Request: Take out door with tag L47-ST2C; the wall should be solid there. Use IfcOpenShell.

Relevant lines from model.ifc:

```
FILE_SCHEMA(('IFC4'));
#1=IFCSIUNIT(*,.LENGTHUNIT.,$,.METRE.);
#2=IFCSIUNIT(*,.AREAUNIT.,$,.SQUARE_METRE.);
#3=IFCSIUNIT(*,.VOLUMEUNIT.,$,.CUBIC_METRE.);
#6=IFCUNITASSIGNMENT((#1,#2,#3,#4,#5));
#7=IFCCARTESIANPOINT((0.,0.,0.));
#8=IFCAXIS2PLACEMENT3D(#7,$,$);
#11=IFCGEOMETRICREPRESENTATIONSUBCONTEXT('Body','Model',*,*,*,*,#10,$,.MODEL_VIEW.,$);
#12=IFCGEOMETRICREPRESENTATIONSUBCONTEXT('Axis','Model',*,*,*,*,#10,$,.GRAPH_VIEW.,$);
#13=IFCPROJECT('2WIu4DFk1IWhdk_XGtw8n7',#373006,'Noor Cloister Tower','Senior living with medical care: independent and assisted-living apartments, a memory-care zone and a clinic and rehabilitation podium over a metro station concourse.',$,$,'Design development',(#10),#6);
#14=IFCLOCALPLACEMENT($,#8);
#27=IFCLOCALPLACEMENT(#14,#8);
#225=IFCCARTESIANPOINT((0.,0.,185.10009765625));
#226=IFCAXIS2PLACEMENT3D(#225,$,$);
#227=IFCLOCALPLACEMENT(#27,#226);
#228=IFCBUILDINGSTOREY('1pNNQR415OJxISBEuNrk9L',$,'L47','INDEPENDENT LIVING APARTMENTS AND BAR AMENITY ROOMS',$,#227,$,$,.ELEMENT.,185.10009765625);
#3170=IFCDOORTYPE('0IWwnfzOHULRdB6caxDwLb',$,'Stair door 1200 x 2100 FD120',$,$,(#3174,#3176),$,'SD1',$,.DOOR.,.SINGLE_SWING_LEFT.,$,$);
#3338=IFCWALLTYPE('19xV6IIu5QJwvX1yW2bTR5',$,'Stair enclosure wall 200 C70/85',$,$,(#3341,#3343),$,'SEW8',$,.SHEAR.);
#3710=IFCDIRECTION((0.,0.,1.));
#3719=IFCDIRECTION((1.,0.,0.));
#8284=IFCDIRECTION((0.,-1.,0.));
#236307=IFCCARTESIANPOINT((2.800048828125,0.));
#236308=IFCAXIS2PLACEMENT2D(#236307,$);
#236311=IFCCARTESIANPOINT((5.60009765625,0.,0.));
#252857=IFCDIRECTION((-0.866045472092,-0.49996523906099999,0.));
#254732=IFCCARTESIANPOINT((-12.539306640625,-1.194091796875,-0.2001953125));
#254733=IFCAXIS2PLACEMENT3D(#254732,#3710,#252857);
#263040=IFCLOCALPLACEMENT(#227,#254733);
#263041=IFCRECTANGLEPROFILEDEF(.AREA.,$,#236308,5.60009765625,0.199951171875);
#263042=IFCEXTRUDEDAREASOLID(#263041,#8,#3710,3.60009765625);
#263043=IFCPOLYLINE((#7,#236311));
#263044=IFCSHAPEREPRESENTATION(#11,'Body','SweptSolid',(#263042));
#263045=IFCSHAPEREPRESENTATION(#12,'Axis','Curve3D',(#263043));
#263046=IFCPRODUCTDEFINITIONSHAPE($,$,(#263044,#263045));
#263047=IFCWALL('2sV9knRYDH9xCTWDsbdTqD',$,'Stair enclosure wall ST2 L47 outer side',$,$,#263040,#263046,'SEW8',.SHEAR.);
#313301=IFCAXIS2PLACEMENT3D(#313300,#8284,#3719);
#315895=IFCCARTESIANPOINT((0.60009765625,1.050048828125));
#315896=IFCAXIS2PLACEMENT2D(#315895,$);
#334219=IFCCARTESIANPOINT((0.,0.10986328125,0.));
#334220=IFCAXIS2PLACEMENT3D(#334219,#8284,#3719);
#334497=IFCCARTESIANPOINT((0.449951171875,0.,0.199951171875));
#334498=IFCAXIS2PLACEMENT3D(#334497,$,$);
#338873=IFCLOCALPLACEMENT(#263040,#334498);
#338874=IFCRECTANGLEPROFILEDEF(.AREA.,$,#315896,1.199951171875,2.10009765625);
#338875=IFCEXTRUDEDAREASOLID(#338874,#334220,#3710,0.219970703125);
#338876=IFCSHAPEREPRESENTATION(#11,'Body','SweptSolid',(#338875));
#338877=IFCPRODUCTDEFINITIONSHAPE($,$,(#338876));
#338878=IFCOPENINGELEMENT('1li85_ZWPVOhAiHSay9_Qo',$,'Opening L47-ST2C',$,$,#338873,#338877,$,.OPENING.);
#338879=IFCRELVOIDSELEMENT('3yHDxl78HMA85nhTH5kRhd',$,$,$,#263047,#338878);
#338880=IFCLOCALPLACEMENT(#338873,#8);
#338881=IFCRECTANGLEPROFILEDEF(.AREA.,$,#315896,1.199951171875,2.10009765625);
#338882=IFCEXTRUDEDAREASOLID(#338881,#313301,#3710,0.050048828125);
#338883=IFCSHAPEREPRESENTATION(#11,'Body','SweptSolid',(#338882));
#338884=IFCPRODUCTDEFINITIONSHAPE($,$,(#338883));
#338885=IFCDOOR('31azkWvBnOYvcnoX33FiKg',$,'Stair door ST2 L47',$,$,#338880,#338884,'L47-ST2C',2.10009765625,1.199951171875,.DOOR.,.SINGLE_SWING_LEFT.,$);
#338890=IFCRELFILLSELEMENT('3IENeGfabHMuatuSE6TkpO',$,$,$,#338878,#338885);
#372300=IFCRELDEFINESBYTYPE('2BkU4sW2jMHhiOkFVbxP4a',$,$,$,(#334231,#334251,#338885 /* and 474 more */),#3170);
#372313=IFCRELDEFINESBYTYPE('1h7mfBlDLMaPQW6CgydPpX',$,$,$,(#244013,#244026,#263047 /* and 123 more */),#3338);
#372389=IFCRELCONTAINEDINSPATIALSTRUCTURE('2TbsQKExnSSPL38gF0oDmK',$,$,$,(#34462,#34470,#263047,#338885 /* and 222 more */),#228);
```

```python
import ifcopenshell
import ifcopenshell.api.feature
import ifcopenshell.api.root
import ifcopenshell.geom
import ifcopenshell.util.shape

model = ifcopenshell.open("model.ifc")
settings = ifcopenshell.geom.settings()


def volume(element):
    """Net volume in cubic metres, openings subtracted."""
    shape = ifcopenshell.geom.create_shape(settings, element)
    return ifcopenshell.util.shape.get_volume(shape.geometry)


door = model.by_id(338885)
opening = door.FillsVoids[0].RelatingOpeningElement
wall = opening.VoidsElements[0].RelatingBuildingElement
before = volume(wall)

ifcopenshell.api.root.remove_product(model, product=door)
ifcopenshell.api.feature.remove_feature(model, feature=opening)

after = volume(wall)

print(f"wall volume {before:.3f} -> {after:.3f} m3")

model.write("model_rev.ifc")
```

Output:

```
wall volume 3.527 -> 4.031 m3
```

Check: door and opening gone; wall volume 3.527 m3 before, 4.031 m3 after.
